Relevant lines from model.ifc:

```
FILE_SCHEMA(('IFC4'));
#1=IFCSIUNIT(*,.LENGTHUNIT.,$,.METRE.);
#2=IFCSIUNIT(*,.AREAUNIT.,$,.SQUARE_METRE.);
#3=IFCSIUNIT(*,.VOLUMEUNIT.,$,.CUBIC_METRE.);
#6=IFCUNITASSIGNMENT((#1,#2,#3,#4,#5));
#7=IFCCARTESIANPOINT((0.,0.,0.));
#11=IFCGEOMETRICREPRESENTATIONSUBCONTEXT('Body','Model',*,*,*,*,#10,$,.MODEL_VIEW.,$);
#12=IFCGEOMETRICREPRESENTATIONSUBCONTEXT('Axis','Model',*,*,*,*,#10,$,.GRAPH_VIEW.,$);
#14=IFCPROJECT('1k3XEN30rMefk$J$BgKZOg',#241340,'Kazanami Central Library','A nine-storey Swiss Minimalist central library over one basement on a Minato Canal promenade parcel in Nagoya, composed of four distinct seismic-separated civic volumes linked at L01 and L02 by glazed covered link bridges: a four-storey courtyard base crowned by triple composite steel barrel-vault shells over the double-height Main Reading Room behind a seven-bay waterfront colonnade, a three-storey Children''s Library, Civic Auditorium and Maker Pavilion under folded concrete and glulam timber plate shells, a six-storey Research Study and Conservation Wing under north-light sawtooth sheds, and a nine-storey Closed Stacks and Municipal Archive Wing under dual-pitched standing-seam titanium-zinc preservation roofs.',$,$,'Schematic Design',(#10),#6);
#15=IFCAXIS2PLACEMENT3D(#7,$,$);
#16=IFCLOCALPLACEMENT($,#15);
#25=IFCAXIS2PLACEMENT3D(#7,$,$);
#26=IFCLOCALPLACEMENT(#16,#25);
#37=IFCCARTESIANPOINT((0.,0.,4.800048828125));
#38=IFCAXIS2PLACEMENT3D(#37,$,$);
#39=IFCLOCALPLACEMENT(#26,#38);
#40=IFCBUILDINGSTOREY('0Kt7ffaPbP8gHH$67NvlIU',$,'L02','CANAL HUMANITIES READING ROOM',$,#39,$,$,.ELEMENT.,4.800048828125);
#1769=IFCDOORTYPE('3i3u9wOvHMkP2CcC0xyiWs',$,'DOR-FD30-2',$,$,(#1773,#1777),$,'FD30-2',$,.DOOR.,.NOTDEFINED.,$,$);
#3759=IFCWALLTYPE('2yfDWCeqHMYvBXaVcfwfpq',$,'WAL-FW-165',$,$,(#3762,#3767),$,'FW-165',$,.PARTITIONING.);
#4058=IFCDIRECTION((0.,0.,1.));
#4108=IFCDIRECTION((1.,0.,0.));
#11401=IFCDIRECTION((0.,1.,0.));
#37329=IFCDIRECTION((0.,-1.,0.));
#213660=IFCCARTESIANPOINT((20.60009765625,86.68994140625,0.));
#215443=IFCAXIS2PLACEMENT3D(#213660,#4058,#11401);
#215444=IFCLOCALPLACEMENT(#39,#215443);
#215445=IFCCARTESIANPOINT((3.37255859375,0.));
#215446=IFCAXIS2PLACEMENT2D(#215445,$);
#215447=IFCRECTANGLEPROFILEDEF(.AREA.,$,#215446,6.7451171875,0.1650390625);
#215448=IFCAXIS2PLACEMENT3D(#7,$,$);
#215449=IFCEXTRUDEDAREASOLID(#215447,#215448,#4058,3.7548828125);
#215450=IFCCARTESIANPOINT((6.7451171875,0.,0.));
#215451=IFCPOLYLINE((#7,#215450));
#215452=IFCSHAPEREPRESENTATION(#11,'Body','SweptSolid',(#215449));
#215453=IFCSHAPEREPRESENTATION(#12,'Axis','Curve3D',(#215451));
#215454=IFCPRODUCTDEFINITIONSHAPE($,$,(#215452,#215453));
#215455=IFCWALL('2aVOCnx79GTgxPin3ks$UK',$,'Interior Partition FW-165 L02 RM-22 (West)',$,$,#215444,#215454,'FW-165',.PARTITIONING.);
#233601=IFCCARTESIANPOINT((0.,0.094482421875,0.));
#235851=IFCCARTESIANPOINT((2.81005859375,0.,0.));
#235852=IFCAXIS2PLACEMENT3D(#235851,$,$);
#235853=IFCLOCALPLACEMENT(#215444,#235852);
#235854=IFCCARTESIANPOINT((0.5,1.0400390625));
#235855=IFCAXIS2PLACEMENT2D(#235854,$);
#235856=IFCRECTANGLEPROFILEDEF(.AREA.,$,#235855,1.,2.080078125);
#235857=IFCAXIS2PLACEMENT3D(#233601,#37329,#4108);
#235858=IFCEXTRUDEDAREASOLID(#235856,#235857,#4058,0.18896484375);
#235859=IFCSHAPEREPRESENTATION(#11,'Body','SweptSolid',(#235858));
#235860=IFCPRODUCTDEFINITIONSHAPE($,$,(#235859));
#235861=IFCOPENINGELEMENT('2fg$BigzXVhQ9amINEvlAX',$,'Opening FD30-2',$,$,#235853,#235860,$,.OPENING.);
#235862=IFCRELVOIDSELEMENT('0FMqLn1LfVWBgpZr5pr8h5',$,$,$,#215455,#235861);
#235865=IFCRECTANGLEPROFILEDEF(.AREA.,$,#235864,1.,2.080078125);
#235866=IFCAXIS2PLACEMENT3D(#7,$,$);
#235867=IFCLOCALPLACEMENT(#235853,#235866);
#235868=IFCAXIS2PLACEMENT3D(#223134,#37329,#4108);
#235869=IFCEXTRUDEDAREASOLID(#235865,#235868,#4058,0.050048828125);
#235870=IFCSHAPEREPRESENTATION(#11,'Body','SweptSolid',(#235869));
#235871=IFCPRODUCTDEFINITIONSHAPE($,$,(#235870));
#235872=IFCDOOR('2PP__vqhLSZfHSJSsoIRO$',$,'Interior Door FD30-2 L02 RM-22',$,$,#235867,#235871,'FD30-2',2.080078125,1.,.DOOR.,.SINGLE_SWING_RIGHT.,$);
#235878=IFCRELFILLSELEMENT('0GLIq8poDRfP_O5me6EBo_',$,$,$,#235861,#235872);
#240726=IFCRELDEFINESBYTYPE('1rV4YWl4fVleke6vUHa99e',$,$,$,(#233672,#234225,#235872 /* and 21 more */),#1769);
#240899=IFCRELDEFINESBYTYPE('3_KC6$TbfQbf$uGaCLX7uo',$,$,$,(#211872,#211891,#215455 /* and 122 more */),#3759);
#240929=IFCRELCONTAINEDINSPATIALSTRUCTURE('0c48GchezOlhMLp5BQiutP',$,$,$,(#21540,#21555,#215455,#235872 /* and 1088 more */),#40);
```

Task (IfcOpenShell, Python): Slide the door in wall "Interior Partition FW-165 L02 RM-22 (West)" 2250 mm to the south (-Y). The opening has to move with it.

```python
import ifcopenshell
import ifcopenshell.api.geometry
import ifcopenshell.util.placement

model = ifcopenshell.open("model.ifc")

door = model.by_guid("2PP__vqhLSZfHSJSsoIRO$")
opening = door.FillsVoids[0].RelatingOpeningElement
wall = opening.VoidsElements[0].RelatingBuildingElement

wall_matrix = ifcopenshell.util.placement.get_local_placement(wall.ObjectPlacement)
shift = wall_matrix[:3, 0] * -2.25
before = ifcopenshell.util.placement.get_local_placement(door.ObjectPlacement)[:3, 3].copy()

# The door is placed relative to its opening, so it follows when the opening moves.
matrix = ifcopenshell.util.placement.get_local_placement(opening.ObjectPlacement)
matrix[:3, 3] += shift
ifcopenshell.api.geometry.edit_object_placement(
    model, product=opening, matrix=matrix, is_si=False, should_transform_children=True
)

after = ifcopenshell.util.placement.get_local_placement(door.ObjectPlacement)[:3, 3]
print("door moved by", (after - before).round(3) + 0.0)

model.write("model_updated.ifc")
```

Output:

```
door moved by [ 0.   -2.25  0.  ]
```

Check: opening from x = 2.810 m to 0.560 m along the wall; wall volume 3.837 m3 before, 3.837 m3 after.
